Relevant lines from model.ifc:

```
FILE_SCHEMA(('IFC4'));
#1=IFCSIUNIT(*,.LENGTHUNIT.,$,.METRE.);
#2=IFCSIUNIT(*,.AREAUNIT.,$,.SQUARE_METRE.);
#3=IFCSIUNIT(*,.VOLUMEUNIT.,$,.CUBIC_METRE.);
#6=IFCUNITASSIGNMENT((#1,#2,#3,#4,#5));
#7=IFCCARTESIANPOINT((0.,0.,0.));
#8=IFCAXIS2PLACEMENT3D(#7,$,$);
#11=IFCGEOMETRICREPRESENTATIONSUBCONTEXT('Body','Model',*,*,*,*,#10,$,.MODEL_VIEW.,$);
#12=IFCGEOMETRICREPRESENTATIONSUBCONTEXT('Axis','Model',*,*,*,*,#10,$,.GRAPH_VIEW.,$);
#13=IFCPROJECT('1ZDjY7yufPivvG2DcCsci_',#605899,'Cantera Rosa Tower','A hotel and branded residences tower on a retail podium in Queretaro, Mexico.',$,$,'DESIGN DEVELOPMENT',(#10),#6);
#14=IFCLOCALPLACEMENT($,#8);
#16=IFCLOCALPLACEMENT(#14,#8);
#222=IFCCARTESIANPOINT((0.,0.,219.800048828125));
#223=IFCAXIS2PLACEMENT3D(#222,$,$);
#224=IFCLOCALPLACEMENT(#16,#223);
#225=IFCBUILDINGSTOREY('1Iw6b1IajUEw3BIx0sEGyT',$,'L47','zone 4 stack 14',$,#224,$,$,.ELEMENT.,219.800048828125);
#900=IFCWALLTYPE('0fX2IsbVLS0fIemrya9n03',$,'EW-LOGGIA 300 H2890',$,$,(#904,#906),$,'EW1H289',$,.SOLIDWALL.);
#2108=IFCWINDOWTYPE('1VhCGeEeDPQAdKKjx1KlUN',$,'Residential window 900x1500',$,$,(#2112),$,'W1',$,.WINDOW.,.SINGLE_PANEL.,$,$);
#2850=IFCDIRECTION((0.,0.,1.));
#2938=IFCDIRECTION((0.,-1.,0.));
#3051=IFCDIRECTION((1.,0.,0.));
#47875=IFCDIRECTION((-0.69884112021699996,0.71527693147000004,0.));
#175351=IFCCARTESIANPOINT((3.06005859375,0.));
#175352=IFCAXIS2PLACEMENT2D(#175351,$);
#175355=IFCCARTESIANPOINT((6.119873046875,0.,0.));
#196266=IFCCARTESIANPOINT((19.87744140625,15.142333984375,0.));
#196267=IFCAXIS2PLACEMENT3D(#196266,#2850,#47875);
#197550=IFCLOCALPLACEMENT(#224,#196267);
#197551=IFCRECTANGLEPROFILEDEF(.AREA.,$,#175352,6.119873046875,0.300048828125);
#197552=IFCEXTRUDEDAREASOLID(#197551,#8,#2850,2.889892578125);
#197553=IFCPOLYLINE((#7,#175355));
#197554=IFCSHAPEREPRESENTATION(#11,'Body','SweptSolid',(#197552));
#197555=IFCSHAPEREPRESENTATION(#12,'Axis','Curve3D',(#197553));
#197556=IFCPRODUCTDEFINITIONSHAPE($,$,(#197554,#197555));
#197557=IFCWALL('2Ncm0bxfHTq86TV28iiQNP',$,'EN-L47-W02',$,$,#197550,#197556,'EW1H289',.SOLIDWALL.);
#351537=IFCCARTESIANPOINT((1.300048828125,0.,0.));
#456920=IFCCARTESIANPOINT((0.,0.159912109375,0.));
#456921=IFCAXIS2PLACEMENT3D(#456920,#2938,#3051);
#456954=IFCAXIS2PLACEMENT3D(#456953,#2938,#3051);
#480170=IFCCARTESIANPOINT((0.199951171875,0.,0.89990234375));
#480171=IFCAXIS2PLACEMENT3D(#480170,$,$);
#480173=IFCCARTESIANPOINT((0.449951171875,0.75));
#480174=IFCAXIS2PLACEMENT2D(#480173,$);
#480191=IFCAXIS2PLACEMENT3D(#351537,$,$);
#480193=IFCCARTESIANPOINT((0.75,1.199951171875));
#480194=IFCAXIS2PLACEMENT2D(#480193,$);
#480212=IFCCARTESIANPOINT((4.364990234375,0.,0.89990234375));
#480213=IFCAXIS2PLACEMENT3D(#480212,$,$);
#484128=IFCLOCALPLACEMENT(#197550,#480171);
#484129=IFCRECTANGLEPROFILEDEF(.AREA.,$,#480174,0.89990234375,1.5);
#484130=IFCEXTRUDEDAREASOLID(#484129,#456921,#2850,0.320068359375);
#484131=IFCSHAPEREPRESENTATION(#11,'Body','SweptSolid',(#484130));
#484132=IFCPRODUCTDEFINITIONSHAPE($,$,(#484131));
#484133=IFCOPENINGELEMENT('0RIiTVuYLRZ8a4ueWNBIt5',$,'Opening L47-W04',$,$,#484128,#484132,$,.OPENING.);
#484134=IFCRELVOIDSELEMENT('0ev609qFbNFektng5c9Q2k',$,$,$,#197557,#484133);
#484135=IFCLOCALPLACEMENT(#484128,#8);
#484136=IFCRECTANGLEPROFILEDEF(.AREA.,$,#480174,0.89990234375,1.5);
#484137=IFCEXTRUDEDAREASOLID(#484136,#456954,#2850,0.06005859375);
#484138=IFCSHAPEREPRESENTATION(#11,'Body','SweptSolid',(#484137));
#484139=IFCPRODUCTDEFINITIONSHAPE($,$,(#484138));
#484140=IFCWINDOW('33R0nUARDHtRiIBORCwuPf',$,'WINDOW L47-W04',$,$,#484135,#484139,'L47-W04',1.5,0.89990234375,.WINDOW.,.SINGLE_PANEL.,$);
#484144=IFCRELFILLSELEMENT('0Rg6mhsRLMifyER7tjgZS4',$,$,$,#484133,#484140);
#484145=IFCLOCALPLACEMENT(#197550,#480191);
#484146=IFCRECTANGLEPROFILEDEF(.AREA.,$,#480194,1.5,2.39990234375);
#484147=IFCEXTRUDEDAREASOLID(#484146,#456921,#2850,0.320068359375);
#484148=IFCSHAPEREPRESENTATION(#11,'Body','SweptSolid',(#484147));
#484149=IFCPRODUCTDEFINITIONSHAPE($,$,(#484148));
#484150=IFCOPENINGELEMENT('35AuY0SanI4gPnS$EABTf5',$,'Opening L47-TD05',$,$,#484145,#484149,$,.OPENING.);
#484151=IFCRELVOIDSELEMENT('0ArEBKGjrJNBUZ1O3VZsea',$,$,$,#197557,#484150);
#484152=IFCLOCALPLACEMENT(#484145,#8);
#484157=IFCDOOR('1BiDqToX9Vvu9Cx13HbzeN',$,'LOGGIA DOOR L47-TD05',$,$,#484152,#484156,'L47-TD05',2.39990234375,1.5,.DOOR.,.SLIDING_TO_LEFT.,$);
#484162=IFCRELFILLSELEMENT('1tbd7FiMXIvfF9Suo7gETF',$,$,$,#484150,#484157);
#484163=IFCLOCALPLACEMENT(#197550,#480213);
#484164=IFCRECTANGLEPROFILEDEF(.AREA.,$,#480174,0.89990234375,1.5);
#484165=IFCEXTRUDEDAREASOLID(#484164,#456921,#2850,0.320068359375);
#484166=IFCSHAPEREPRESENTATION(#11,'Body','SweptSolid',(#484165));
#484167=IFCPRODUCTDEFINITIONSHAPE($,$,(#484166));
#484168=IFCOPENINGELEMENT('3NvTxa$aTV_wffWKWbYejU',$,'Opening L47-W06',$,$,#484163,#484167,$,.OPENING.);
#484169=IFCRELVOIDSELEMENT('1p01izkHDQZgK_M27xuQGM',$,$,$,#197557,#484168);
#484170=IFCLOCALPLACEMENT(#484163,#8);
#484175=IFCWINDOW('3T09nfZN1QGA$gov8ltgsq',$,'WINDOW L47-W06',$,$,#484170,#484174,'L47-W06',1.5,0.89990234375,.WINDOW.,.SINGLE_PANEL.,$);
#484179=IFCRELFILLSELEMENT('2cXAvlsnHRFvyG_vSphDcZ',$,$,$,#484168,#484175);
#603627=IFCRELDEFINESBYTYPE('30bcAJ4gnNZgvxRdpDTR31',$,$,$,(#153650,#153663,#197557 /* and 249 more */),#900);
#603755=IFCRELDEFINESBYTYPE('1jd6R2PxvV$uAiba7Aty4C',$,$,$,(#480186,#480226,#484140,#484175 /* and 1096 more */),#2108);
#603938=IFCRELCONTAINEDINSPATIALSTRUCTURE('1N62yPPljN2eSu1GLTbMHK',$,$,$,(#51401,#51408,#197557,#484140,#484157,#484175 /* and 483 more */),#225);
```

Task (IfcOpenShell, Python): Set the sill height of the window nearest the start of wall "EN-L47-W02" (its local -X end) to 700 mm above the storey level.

```python
import numpy as np
import ifcopenshell
import ifcopenshell.api.geometry
import ifcopenshell.geom
import ifcopenshell.util.element
import ifcopenshell.util.placement
import ifcopenshell.util.shape
import ifcopenshell.util.unit

model = ifcopenshell.open("model.ifc")
unit_scale = ifcopenshell.util.unit.calculate_unit_scale(model)

window = model.by_guid("33R0nUARDHtRiIBORCwuPf")
opening = window.FillsVoids[0].RelatingOpeningElement
storey = ifcopenshell.util.element.get_container(window, ifc_class="IfcBuildingStorey")
level = ifcopenshell.util.placement.get_local_placement(storey.ObjectPlacement)[2, 3]

# The opening's origin need not be at the sill, so measure its lowest point.
shape = ifcopenshell.geom.create_shape(ifcopenshell.geom.settings(), opening)
bottom = ifcopenshell.util.shape.get_shape_bottom_elevation(shape, shape.geometry) / unit_scale
dz = level + 0.7 / unit_scale - bottom

shift = np.array([0.0, 0.0, dz])
# The window is placed relative to its opening, so it follows when the opening moves.
matrix = ifcopenshell.util.placement.get_local_placement(opening.ObjectPlacement)
matrix[:3, 3] += shift
ifcopenshell.api.geometry.edit_object_placement(
    model, product=opening, matrix=matrix, is_si=False, should_transform_children=True
)

print(f"moved by {dz * unit_scale:+.3f} m")

model.write("model-out.ifc")
```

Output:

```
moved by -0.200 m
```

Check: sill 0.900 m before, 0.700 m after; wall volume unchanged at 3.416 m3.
